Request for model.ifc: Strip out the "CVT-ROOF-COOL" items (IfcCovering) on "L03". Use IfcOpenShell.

First a look at what the model holds.

```python
import ifcopenshell
import ifcopenshell.util.element

model = ifcopenshell.open("model.ifc")
print(model.schema)
storey = next(s for s in model.by_type("IfcBuildingStorey") if s.Name == "L03")
coverings = [e for e in ifcopenshell.util.element.get_decomposition(storey) if e.is_a("IfcCovering")]
seen = {}
for e in coverings:
    element_type = ifcopenshell.util.element.get_type(e)
    name = element_type.Name if element_type not in (None, e) else None
    seen[name] = seen.get(name, 0) + 1
for name, count in sorted(seen.items(), key=str):
    print(count, "x", name)
```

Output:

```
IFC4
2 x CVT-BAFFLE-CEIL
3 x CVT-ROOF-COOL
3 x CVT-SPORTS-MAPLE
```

```python
import ifcopenshell
import ifcopenshell.api.root
import ifcopenshell.util.element

model = ifcopenshell.open("model.ifc")

storey = next(s for s in model.by_type("IfcBuildingStorey") if s.Name == "L03")
coverings = [e for e in ifcopenshell.util.element.get_decomposition(storey) if e.is_a("IfcCovering")]
targets = [e for e in coverings if (t := ifcopenshell.util.element.get_type(e)) not in (None, e) and t.Name == "CVT-ROOF-COOL"]

for e in targets:
    ifcopenshell.api.root.remove_product(model, product=e)
print(len(targets), "removed")

model.write("model_rev.ifc")
```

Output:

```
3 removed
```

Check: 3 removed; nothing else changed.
